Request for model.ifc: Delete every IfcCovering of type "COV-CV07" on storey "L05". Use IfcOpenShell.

First a look at what the model holds.

```python
import ifcopenshell
import ifcopenshell.util.element

model = ifcopenshell.open("model.ifc")
print(model.schema)
storey = next(s for s in model.by_type("IfcBuildingStorey") if s.Name == "L05")
coverings = [e for e in ifcopenshell.util.element.get_decomposition(storey) if e.is_a("IfcCovering")]
seen = {}
for e in coverings:
    element_type = ifcopenshell.util.element.get_type(e)
    name = element_type.Name if element_type not in (None, e) else None
    seen[name] = seen.get(name, 0) + 1
for name, count in sorted(seen.items(), key=str):
    print(count, "x", name)
```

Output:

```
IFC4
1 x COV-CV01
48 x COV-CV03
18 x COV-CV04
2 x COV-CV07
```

```python
import ifcopenshell
import ifcopenshell.api.root
import ifcopenshell.util.element

model = ifcopenshell.open("model.ifc")

storey = next(s for s in model.by_type("IfcBuildingStorey") if s.Name == "L05")
coverings = [e for e in ifcopenshell.util.element.get_decomposition(storey) if e.is_a("IfcCovering")]
targets = [e for e in coverings if (t := ifcopenshell.util.element.get_type(e)) not in (None, e) and t.Name == "COV-CV07"]

for e in targets:
    ifcopenshell.api.root.remove_product(model, product=e)
print(len(targets), "removed")

model.write("model_edited.ifc")
```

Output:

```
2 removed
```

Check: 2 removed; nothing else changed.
